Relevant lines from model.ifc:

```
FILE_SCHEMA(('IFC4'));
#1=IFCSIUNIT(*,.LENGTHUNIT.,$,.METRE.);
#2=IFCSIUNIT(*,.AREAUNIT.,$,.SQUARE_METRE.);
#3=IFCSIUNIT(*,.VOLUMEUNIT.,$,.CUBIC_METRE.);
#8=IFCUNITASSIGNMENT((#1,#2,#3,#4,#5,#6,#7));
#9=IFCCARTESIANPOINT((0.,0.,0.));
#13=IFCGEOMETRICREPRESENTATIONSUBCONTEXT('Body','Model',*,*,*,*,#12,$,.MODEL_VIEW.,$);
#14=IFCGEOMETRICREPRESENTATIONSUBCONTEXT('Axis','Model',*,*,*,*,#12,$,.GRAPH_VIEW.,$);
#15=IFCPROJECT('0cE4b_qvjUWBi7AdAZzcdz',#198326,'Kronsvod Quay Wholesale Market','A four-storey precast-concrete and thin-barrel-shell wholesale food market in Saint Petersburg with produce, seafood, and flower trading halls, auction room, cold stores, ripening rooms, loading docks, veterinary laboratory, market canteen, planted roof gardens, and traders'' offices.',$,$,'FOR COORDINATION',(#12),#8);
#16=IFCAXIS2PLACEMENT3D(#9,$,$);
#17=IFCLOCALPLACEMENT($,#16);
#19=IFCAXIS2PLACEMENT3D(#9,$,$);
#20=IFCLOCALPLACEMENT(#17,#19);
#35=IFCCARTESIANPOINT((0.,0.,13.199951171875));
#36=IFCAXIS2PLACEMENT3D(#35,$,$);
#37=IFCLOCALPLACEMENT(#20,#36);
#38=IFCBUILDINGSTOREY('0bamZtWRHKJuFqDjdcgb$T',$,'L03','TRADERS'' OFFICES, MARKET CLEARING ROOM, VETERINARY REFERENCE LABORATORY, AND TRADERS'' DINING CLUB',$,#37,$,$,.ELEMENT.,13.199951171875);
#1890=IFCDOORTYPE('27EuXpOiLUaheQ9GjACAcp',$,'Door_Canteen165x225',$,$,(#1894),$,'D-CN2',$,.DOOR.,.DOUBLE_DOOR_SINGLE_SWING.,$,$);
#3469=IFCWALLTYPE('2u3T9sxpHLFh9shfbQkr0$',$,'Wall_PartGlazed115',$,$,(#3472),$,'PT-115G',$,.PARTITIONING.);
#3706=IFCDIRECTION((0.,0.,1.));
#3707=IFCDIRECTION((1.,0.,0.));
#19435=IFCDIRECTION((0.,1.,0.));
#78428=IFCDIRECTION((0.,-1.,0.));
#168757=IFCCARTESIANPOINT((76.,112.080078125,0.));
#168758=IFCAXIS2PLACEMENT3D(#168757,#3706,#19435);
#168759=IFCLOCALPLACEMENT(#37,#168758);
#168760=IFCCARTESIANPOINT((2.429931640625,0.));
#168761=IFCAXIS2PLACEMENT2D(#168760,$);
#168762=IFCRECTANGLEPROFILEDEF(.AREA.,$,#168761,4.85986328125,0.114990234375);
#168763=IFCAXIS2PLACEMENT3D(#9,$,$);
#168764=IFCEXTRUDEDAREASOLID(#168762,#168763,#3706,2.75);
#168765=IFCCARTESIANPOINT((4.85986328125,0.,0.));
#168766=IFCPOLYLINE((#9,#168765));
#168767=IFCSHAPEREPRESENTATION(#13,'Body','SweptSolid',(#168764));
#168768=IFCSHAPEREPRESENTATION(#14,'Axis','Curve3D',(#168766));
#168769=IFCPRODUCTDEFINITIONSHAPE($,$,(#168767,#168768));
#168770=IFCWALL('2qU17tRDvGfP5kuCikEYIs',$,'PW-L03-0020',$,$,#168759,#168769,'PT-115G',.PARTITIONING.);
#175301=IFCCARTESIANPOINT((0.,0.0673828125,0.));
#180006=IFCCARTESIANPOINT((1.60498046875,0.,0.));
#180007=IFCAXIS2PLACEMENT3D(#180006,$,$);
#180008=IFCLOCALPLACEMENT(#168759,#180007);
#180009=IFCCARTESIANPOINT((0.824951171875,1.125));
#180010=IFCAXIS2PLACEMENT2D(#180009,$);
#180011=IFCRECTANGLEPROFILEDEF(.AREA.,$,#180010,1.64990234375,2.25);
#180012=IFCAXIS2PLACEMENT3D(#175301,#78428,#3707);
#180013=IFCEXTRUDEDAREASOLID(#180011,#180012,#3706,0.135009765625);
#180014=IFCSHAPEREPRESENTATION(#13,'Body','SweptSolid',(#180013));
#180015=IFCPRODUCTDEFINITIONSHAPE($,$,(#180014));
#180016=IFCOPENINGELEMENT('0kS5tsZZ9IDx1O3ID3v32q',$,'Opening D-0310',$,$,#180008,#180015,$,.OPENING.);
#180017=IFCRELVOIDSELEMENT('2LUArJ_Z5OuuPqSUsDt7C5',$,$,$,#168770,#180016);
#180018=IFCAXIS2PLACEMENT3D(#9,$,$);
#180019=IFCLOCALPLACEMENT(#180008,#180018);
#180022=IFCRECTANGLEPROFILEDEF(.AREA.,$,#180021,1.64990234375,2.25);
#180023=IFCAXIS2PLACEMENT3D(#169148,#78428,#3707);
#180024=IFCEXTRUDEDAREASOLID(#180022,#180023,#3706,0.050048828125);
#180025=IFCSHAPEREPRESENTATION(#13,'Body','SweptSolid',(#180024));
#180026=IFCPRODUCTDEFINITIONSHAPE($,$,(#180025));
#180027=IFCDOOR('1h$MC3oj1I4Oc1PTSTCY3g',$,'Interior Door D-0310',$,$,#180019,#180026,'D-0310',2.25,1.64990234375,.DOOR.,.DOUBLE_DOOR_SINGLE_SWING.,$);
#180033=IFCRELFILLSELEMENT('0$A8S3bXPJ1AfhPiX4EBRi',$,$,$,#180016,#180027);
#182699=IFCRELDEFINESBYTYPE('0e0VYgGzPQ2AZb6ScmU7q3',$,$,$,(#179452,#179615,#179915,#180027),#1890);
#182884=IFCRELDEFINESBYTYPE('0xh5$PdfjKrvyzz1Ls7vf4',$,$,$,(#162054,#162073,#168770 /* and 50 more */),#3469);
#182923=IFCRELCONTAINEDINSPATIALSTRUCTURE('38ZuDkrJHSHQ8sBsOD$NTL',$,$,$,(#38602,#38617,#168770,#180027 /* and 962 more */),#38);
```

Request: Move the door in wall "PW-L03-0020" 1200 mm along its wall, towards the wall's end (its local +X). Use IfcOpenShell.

```python
import ifcopenshell
import ifcopenshell.api.geometry
import ifcopenshell.util.placement
import ifcopenshell.util.unit

model = ifcopenshell.open("model.ifc")
unit_scale = ifcopenshell.util.unit.calculate_unit_scale(model)

door = model.by_guid("1h$MC3oj1I4Oc1PTSTCY3g")
opening = door.FillsVoids[0].RelatingOpeningElement
wall = opening.VoidsElements[0].RelatingBuildingElement

wall_matrix = ifcopenshell.util.placement.get_local_placement(wall.ObjectPlacement)
shift = wall_matrix[:3, 0] * 1.2 / unit_scale
before = ifcopenshell.util.placement.get_local_placement(door.ObjectPlacement)[:3, 3].copy()

# The door is placed relative to its opening, so it follows when the opening moves.
matrix = ifcopenshell.util.placement.get_local_placement(opening.ObjectPlacement)
matrix[:3, 3] += shift
ifcopenshell.api.geometry.edit_object_placement(
    model, product=opening, matrix=matrix, is_si=False, should_transform_children=True
)

after = ifcopenshell.util.placement.get_local_placement(door.ObjectPlacement)[:3, 3]
print("door moved by", (after - before).round(3) + 0.0)

model.write("model_v2.ifc")
```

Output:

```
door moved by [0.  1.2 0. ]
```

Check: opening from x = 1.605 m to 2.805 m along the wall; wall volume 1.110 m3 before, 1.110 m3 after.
